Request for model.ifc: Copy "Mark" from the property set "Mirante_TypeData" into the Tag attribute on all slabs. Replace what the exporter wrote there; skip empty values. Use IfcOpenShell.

First a look at what the model holds.

```python
import ifcopenshell
import ifcopenshell.util.element

model = ifcopenshell.open("model.ifc")
print(model.schema)
slabs = model.by_type("IfcSlab")
print(len(slabs), "slabs")
for e in slabs[:8]:
    source = ifcopenshell.util.element.get_pset(e, "Mirante_TypeData", "Mark")
    target = e.Tag
    print(e.id(), repr(source), repr(target), sep=" | ")
```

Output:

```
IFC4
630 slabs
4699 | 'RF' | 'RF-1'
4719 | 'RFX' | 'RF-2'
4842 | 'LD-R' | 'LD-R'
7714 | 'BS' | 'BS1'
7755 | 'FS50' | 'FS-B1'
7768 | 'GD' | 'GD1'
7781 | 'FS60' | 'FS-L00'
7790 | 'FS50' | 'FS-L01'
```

```python
import ifcopenshell
import ifcopenshell.util.element

model = ifcopenshell.open("model.ifc")

count = 0
for e in model.by_type("IfcSlab"):
    value = ifcopenshell.util.element.get_pset(e, "Mirante_TypeData", "Mark")
    current = e.Tag
    if not value or not value.strip() or current == value:
        continue
    e.Tag = value
    count += 1

print(count, "slabs updated")

model.write("model_rev.ifc")
```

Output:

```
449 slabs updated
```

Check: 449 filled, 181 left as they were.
